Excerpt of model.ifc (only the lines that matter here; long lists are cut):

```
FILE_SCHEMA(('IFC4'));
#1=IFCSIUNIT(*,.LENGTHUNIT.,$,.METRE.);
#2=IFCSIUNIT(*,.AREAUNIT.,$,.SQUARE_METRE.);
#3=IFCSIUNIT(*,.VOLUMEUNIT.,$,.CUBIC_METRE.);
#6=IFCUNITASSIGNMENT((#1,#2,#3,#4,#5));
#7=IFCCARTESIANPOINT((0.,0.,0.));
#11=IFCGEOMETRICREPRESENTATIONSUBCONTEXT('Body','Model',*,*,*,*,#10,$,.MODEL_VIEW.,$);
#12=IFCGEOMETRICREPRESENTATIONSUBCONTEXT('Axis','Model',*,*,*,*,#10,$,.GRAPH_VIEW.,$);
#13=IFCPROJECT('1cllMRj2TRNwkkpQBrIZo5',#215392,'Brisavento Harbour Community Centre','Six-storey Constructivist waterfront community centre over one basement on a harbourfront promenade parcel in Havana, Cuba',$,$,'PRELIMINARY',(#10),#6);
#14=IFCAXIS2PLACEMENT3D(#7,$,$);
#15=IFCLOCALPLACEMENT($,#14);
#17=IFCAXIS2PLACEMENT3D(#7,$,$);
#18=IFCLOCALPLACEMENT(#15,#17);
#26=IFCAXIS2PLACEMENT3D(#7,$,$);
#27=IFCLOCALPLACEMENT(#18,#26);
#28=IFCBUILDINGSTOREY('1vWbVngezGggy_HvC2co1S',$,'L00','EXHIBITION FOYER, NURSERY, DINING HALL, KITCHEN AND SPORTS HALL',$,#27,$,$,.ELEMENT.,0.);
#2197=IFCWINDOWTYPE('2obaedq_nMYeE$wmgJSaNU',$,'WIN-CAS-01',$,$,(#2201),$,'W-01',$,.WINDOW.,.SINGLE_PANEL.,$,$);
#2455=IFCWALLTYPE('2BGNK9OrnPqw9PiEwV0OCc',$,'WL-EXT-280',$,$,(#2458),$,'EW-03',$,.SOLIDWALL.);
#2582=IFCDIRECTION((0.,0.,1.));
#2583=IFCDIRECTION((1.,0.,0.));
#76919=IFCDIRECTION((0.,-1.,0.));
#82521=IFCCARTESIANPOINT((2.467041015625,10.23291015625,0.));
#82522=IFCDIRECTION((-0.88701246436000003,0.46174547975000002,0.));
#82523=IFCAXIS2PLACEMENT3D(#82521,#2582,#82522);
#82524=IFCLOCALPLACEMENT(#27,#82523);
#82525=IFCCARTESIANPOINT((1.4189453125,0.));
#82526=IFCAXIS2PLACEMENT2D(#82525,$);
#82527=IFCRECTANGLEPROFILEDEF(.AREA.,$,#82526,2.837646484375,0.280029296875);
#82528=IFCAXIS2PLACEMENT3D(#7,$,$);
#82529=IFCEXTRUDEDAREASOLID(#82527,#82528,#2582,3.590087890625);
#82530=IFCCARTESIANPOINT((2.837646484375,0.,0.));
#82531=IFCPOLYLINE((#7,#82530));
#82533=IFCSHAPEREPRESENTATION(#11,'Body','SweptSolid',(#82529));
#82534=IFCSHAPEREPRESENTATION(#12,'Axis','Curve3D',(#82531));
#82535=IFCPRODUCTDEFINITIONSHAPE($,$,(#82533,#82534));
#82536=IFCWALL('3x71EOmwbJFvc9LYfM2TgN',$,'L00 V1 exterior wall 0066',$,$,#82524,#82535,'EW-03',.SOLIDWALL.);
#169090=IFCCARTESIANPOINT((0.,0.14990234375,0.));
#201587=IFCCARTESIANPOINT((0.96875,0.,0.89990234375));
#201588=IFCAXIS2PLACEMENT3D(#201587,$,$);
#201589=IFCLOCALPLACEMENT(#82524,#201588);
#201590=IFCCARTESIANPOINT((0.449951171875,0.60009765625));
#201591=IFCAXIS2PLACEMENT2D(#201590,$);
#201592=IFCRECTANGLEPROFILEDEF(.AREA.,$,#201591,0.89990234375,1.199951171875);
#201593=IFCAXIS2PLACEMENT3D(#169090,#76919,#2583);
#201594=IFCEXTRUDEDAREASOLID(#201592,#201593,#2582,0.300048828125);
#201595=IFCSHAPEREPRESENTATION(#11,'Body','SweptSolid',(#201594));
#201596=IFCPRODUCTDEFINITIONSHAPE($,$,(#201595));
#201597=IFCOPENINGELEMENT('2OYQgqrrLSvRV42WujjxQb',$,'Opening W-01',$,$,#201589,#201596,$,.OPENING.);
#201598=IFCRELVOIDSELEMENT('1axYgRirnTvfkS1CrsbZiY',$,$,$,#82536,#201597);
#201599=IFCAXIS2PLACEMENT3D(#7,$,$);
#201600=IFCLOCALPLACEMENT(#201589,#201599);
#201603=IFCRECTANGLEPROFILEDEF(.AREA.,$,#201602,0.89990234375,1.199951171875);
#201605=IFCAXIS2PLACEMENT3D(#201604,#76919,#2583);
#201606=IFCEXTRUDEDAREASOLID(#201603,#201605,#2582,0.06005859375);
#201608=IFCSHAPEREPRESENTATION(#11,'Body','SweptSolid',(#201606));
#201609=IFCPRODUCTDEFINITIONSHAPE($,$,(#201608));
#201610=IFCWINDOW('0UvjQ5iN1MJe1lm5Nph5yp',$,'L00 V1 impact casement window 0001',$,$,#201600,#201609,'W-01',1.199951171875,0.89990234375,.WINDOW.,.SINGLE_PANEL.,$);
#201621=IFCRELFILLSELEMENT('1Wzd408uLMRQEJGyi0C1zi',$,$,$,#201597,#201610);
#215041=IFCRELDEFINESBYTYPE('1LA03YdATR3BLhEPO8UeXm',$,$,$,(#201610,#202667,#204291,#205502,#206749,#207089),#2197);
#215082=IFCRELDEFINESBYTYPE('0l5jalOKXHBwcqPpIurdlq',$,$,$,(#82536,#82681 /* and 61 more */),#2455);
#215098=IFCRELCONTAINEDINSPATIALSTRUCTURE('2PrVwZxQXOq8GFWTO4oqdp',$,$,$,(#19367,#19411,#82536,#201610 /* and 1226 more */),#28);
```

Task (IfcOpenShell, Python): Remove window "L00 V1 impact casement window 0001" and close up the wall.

```python
import ifcopenshell
import ifcopenshell.api.feature
import ifcopenshell.api.root
import ifcopenshell.geom
import ifcopenshell.util.shape

model = ifcopenshell.open("model.ifc")
settings = ifcopenshell.geom.settings()


def volume(element):
    """Net volume in cubic metres, openings subtracted."""
    shape = ifcopenshell.geom.create_shape(settings, element)
    return ifcopenshell.util.shape.get_volume(shape.geometry)


window = model.by_guid("0UvjQ5iN1MJe1lm5Nph5yp")
opening = window.FillsVoids[0].RelatingOpeningElement
wall = opening.VoidsElements[0].RelatingBuildingElement
before = volume(wall)

ifcopenshell.api.root.remove_product(model, product=window)
ifcopenshell.api.feature.remove_feature(model, feature=opening)

after = volume(wall)

print(f"wall volume {before:.3f} -> {after:.3f} m3")

model.write("model_v2.ifc")
```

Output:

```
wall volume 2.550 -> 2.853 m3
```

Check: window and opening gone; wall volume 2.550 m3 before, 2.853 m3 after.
